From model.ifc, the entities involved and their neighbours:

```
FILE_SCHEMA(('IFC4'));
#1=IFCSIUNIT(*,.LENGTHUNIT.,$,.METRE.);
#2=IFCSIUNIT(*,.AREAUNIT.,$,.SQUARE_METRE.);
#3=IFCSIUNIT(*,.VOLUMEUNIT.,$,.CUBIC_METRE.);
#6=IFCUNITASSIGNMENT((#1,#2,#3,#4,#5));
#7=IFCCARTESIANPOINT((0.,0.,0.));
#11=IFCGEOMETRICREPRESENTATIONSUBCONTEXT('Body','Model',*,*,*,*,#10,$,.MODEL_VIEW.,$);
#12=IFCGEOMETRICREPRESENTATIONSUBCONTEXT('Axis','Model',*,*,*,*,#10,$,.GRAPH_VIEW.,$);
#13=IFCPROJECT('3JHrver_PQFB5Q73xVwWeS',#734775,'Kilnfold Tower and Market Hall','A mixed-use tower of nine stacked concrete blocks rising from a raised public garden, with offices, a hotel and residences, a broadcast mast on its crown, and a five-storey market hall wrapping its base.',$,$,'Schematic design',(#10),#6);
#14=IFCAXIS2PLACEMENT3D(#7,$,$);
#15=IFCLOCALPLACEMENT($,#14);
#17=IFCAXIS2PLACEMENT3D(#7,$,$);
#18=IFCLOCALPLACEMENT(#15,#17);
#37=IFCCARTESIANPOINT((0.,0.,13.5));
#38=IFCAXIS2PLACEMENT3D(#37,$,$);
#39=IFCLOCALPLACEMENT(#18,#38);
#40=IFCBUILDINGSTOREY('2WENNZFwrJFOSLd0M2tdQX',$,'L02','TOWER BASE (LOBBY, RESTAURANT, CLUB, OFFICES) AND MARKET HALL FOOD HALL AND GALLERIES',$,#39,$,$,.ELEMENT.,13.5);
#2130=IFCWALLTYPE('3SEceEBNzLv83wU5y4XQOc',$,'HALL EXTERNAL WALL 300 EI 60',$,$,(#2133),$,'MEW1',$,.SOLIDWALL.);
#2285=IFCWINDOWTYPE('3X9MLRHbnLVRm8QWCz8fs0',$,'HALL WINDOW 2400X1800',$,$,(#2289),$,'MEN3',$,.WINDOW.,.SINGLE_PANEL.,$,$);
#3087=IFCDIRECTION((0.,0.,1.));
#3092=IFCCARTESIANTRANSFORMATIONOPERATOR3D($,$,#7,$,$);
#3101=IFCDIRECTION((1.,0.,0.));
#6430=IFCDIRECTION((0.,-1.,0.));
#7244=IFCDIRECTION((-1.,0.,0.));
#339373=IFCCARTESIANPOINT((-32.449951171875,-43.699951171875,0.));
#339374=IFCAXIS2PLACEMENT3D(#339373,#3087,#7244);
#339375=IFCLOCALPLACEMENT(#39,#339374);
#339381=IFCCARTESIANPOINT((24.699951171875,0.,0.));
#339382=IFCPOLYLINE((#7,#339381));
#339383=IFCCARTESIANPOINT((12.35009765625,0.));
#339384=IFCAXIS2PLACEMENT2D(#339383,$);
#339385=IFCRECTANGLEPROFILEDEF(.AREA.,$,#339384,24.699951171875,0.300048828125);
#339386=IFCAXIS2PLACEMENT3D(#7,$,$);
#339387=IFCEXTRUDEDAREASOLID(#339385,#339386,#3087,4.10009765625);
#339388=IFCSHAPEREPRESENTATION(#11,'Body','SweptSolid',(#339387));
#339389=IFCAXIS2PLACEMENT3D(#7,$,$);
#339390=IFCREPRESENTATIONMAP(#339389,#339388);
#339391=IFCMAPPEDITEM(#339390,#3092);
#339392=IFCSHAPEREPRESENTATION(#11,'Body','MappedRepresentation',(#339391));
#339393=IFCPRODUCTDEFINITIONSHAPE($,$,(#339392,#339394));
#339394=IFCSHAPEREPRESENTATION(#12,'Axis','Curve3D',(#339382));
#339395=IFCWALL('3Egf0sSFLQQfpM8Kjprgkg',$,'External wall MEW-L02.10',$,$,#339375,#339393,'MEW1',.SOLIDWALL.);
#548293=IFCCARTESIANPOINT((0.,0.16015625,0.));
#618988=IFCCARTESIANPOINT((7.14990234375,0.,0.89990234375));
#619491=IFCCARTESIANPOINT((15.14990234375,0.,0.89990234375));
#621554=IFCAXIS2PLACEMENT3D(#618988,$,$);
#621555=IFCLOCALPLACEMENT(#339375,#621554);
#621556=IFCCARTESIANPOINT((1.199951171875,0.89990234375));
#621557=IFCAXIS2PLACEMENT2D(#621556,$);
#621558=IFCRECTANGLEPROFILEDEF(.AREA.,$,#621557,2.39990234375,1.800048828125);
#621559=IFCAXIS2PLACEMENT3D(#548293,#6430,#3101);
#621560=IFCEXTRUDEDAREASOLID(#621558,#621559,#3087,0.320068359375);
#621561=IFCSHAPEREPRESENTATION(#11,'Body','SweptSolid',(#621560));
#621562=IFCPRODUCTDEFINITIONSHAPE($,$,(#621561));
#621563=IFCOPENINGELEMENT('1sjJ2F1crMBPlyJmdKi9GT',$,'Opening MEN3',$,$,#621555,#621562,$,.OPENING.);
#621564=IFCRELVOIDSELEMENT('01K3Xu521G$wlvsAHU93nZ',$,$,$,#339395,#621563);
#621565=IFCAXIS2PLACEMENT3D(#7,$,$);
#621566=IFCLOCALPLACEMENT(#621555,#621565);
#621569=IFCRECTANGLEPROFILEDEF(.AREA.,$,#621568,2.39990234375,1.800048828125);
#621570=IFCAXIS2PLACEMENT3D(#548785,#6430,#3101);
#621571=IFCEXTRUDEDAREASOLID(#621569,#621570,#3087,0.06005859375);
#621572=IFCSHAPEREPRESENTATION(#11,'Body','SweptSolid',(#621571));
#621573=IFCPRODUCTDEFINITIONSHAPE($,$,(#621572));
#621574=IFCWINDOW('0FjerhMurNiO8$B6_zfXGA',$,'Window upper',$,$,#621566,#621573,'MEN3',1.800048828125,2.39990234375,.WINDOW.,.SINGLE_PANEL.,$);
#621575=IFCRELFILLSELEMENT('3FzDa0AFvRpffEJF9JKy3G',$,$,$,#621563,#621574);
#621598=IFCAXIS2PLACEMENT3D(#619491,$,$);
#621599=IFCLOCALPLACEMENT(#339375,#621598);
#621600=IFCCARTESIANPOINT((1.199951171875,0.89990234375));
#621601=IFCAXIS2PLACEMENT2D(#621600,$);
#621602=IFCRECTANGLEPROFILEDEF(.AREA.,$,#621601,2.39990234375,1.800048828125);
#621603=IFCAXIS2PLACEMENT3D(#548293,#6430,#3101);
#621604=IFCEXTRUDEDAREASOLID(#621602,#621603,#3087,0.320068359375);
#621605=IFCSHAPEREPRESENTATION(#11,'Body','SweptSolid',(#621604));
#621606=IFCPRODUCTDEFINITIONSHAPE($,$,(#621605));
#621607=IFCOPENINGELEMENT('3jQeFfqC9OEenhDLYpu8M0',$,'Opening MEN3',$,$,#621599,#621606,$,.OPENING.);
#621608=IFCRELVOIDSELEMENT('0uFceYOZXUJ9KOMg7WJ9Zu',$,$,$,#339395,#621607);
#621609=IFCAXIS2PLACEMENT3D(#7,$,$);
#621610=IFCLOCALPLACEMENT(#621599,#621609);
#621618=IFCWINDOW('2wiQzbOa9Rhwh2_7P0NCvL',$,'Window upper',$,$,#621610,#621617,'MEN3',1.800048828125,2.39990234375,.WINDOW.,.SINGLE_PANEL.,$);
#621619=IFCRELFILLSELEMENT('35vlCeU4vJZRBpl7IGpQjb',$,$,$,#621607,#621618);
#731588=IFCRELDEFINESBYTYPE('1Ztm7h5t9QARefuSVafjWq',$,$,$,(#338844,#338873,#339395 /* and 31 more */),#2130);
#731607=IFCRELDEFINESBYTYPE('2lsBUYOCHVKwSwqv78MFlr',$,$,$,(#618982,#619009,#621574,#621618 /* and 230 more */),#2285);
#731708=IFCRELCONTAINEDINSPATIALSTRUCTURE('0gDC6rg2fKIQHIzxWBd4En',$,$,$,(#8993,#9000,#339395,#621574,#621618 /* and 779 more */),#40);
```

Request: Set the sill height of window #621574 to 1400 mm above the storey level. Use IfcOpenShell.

```python
import numpy as np
import ifcopenshell
import ifcopenshell.api.geometry
import ifcopenshell.geom
import ifcopenshell.util.element
import ifcopenshell.util.placement
import ifcopenshell.util.shape
import ifcopenshell.util.unit

model = ifcopenshell.open("model.ifc")
unit_scale = ifcopenshell.util.unit.calculate_unit_scale(model)

window = model.by_guid("0FjerhMurNiO8$B6_zfXGA")
opening = window.FillsVoids[0].RelatingOpeningElement
storey = ifcopenshell.util.element.get_container(window, ifc_class="IfcBuildingStorey")
level = ifcopenshell.util.placement.get_local_placement(storey.ObjectPlacement)[2, 3]

# The opening's origin need not be at the sill, so measure its lowest point.
shape = ifcopenshell.geom.create_shape(ifcopenshell.geom.settings(), opening)
bottom = ifcopenshell.util.shape.get_shape_bottom_elevation(shape, shape.geometry) / unit_scale
dz = level + 1.4 - bottom

shift = np.array([0.0, 0.0, dz])
# The window is placed relative to its opening, so it follows when the opening moves.
matrix = ifcopenshell.util.placement.get_local_placement(opening.ObjectPlacement)
matrix[:3, 3] += shift
ifcopenshell.api.geometry.edit_object_placement(
    model, product=opening, matrix=matrix, is_si=False, should_transform_children=True
)

print(f"moved by {dz * unit_scale:+.3f} m")

model.write("model_edited.ifc")
```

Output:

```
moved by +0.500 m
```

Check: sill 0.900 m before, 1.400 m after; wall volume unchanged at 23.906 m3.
